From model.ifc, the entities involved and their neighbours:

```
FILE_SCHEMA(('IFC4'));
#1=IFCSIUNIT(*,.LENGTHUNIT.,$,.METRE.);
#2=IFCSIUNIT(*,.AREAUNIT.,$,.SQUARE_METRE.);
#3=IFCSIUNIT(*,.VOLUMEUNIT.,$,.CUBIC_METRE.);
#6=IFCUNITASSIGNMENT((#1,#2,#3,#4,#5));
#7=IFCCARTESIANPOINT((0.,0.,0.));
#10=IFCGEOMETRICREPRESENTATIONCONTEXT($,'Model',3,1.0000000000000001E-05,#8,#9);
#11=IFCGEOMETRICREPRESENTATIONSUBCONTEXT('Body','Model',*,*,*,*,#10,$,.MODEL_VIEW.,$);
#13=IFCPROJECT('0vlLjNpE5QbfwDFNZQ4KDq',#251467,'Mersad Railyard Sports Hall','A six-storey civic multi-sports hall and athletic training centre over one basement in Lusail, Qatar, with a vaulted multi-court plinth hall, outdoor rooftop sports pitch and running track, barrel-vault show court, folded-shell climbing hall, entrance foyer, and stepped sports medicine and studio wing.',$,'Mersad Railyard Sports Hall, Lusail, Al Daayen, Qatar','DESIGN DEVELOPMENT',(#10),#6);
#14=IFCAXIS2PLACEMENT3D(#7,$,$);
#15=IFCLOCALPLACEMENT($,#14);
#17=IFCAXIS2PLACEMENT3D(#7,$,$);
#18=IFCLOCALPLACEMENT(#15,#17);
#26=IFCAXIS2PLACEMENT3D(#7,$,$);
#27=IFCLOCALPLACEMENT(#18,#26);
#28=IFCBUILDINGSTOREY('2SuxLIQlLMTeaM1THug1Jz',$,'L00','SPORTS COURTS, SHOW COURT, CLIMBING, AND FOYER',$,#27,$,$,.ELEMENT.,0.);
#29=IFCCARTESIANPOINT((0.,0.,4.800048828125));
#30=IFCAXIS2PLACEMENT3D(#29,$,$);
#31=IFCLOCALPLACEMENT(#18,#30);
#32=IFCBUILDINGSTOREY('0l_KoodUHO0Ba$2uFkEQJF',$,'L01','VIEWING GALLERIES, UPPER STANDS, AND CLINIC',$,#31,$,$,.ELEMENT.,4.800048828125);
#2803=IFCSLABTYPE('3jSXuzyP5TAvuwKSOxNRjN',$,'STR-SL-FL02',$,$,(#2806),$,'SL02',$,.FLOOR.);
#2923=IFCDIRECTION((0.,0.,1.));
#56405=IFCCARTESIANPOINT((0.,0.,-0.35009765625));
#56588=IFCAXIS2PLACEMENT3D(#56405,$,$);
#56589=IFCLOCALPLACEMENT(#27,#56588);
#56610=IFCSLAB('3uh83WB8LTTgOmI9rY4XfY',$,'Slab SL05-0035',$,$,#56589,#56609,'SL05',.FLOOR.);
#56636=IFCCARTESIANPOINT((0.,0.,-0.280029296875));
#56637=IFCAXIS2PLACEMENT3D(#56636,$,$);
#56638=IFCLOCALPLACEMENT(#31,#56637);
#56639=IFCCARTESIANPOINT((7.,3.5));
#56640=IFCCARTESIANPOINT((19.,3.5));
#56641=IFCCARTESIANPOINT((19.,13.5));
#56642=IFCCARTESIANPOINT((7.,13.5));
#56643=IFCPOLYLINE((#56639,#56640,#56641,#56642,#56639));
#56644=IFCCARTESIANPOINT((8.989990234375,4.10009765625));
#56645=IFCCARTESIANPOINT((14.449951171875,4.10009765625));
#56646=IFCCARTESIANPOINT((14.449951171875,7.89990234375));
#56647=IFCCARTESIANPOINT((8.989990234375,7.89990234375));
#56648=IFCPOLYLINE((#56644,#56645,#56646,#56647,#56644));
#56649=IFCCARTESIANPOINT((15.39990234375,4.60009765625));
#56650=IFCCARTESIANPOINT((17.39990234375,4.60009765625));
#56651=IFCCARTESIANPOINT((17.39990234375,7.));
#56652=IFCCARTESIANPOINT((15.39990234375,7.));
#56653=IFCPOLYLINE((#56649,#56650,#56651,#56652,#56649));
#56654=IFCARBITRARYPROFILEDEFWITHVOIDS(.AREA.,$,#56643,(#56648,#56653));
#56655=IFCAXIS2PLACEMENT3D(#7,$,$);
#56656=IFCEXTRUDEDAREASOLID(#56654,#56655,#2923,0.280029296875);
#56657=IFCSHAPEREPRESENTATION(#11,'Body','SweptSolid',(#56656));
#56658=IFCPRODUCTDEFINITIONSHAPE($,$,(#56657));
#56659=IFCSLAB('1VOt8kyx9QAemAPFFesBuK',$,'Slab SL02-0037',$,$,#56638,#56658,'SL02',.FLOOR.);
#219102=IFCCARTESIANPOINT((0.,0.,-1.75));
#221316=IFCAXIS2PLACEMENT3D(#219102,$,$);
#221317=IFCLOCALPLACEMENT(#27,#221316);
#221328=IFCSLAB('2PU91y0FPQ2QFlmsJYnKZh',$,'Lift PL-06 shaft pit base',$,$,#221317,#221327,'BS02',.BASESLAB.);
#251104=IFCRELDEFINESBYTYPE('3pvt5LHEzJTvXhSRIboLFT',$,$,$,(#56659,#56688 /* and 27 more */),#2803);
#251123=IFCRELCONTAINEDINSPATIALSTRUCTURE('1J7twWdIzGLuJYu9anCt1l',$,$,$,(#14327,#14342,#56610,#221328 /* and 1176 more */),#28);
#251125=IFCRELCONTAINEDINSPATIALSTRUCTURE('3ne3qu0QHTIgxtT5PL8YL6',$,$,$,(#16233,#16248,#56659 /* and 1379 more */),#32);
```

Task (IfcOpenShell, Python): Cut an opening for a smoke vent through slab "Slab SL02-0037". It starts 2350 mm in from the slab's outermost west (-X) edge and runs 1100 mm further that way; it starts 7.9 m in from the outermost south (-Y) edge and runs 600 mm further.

```python
import numpy as np
import ifcopenshell
import ifcopenshell.api.feature
import ifcopenshell.api.geometry
import ifcopenshell.api.root
import ifcopenshell.geom
import ifcopenshell.util.placement
import ifcopenshell.util.representation
import ifcopenshell.util.shape
import ifcopenshell.util.unit

model = ifcopenshell.open("model.ifc")
unit_scale = ifcopenshell.util.unit.calculate_unit_scale(model)
settings = ifcopenshell.geom.settings()


def volume(element):
    """Net volume in cubic metres, openings subtracted."""
    shape = ifcopenshell.geom.create_shape(settings, element)
    return ifcopenshell.util.shape.get_volume(shape.geometry)


slab = model.by_guid("1VOt8kyx9QAemAPFFesBuK")
before = volume(slab)

# Extent in the slab's own axes, in metres. The edges named are its -X and -Y sides.
slab_shape = ifcopenshell.geom.create_shape(settings, slab)
vertices = ifcopenshell.util.shape.get_vertices(slab_shape.geometry)
x_min, y_min, bottom = vertices.min(axis=0)
top = vertices[:, 2].max()

opening = ifcopenshell.api.root.create_entity(model, ifc_class="IfcOpeningElement", name="Smoke vent opening", predefined_type="OPENING")
context = ifcopenshell.util.representation.get_context(model, "Model", "Body", "MODEL_VIEW")
width, depth = 1.1, 0.6
outline = [(0.0, 0.0), (width, 0.0), (width, depth), (0.0, depth), (0.0, 0.0)]
# Overshoot both faces by 50 mm so the cut is clean.
shape = ifcopenshell.api.geometry.add_slab_representation(
    model, context=context, depth=top - bottom + 0.1, polyline=outline
)
ifcopenshell.api.geometry.assign_representation(model, product=opening, representation=shape)

matrix = ifcopenshell.util.placement.get_local_placement(slab.ObjectPlacement)
matrix[:, 3] = matrix @ np.append(np.array([x_min + 2.35, y_min + 7.9, bottom - 0.05]) / unit_scale, 1.0)
ifcopenshell.api.geometry.edit_object_placement(model, product=opening, matrix=matrix, is_si=False)
ifcopenshell.api.feature.add_feature(model, feature=opening, element=slab)

after = volume(slab)

print(f"slab volume {before:.3f} -> {after:.3f} m3")

model.write("model-out.ifc")
```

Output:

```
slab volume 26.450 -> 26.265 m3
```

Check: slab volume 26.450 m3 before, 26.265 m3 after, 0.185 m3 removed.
